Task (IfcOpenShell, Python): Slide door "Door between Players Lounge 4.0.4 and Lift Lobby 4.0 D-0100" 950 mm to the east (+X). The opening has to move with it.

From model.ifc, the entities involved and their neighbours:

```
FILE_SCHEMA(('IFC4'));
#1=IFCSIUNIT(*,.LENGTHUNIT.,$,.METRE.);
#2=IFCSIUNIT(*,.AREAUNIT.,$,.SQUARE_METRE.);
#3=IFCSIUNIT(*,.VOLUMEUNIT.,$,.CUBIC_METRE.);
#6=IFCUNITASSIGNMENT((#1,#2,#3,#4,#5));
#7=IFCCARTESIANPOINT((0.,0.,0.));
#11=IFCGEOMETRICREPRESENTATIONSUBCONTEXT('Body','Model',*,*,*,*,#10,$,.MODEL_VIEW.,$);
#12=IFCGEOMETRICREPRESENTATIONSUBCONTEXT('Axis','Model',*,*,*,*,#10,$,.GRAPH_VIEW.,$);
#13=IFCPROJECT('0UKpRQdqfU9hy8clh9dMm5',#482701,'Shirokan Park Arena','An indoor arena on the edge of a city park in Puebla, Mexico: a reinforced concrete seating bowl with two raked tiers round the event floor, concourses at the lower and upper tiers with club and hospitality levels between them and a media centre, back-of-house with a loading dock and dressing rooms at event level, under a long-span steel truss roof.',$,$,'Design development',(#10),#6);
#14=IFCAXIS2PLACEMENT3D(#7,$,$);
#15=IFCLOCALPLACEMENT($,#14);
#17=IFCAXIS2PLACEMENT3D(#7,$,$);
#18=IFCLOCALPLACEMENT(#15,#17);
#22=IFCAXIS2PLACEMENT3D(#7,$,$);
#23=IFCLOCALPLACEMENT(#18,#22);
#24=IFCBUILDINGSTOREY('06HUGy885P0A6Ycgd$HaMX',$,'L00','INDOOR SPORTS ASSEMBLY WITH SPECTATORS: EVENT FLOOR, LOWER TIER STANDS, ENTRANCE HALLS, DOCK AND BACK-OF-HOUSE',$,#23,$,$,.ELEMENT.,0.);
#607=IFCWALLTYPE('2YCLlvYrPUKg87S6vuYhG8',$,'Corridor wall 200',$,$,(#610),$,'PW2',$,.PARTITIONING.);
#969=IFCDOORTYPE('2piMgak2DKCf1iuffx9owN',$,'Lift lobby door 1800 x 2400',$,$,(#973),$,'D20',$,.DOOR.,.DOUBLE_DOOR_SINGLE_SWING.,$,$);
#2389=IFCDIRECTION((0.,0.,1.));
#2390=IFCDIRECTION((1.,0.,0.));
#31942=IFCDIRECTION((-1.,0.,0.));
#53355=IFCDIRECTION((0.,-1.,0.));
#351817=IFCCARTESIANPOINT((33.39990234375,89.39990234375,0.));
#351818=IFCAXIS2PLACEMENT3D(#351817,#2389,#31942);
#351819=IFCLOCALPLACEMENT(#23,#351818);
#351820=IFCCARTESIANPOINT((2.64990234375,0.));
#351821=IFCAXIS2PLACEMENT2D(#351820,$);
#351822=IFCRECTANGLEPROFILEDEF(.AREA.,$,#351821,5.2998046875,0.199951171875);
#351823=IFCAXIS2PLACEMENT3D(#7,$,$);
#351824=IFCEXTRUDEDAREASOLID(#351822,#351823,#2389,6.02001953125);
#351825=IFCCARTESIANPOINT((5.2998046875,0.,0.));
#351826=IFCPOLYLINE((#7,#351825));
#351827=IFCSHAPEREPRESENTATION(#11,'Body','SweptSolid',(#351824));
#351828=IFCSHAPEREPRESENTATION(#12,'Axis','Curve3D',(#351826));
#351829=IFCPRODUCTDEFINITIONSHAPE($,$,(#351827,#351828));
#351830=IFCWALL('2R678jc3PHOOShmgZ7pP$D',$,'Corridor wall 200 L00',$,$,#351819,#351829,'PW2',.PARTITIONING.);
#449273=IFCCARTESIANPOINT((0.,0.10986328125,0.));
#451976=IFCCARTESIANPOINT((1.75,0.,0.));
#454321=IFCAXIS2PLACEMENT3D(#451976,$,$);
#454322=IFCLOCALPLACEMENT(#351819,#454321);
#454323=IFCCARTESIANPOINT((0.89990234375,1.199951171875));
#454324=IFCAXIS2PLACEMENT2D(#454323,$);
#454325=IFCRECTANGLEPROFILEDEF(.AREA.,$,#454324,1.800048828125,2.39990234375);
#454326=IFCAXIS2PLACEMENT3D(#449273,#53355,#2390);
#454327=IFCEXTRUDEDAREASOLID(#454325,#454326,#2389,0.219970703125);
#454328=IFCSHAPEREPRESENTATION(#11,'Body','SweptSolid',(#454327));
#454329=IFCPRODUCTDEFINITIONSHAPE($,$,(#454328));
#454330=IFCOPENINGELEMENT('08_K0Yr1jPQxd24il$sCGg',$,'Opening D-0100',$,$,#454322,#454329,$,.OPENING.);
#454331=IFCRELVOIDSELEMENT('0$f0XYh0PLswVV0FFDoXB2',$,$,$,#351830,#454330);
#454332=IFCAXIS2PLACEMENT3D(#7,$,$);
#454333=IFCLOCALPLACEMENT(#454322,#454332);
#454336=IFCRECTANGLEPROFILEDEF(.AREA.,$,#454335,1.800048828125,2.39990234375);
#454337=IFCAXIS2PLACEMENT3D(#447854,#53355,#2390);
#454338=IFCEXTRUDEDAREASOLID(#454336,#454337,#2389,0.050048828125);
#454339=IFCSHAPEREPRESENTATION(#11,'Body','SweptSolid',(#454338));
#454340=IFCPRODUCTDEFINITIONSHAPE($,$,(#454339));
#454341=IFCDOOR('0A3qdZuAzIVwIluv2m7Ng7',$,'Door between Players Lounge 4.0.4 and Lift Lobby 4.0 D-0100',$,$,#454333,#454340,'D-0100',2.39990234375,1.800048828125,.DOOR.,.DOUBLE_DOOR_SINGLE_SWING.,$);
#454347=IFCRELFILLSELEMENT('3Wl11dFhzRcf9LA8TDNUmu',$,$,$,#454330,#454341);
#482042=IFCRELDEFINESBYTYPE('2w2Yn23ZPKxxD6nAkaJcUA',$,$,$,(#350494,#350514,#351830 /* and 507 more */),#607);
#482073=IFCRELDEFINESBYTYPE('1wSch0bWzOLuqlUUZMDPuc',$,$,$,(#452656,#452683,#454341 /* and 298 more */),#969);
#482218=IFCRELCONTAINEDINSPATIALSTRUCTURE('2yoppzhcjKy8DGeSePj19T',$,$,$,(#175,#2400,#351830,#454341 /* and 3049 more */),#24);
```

```python
import ifcopenshell
import ifcopenshell.api.geometry
import ifcopenshell.util.placement

model = ifcopenshell.open("model.ifc")

door = model.by_guid("0A3qdZuAzIVwIluv2m7Ng7")
opening = door.FillsVoids[0].RelatingOpeningElement
wall = opening.VoidsElements[0].RelatingBuildingElement

wall_matrix = ifcopenshell.util.placement.get_local_placement(wall.ObjectPlacement)
shift = wall_matrix[:3, 0] * -0.95
before = ifcopenshell.util.placement.get_local_placement(door.ObjectPlacement)[:3, 3].copy()

# The door is placed relative to its opening, so it follows when the opening moves.
matrix = ifcopenshell.util.placement.get_local_placement(opening.ObjectPlacement)
matrix[:3, 3] += shift
ifcopenshell.api.geometry.edit_object_placement(
    model, product=opening, matrix=matrix, is_si=False, should_transform_children=True
)

after = ifcopenshell.util.placement.get_local_placement(door.ObjectPlacement)[:3, 3]
print("door moved by", (after - before).round(3) + 0.0)

model.write("model_v2.ifc")
```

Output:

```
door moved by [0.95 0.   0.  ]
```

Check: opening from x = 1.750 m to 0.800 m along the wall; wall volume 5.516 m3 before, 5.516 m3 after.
